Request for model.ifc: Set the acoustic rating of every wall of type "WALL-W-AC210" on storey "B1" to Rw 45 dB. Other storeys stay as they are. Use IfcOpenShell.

First a look at what the model holds.

```python
import ifcopenshell
import ifcopenshell.util.element

model = ifcopenshell.open("model.ifc")
print(model.schema)
storey = next(s for s in model.by_type("IfcBuildingStorey") if s.Name == "B1")
walls = [e for e in ifcopenshell.util.element.get_decomposition(storey) if e.is_a("IfcWall")]
seen = {}
for e in walls:
    element_type = ifcopenshell.util.element.get_type(e)
    key = (element_type.Name if element_type != e and element_type else None, ifcopenshell.util.element.get_pset(e, "Pset_WallCommon", "AcousticRating"))
    seen[key] = seen.get(key, 0) + 1
for (name, value), count in sorted(seen.items(), key=str):
    print(count, "x", name, "|", value)
```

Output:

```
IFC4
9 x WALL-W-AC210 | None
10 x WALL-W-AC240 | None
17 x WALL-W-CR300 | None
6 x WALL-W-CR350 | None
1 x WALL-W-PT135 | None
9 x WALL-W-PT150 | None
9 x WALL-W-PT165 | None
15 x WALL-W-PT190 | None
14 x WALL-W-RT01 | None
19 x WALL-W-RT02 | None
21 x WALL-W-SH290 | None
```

```python
import ifcopenshell
import ifcopenshell.api.pset
import ifcopenshell.util.element

model = ifcopenshell.open("model.ifc")

storey = next(s for s in model.by_type("IfcBuildingStorey") if s.Name == "B1")
walls = [e for e in ifcopenshell.util.element.get_decomposition(storey) if e.is_a("IfcWall")]

count = 0
for e in walls:
    element_type = ifcopenshell.util.element.get_type(e)
    if element_type in (None, e) or element_type.Name != "WALL-W-AC210":
        continue
    # add_pset returns the element's existing set when there is one.
    pset = ifcopenshell.api.pset.add_pset(model, product=e, name="Pset_WallCommon")
    ifcopenshell.api.pset.edit_pset(model, pset=pset, properties={"AcousticRating": "Rw 45 dB"})
    count += 1

print(count, "walls updated")

model.write("model-out.ifc")
```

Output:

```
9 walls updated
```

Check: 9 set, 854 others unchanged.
